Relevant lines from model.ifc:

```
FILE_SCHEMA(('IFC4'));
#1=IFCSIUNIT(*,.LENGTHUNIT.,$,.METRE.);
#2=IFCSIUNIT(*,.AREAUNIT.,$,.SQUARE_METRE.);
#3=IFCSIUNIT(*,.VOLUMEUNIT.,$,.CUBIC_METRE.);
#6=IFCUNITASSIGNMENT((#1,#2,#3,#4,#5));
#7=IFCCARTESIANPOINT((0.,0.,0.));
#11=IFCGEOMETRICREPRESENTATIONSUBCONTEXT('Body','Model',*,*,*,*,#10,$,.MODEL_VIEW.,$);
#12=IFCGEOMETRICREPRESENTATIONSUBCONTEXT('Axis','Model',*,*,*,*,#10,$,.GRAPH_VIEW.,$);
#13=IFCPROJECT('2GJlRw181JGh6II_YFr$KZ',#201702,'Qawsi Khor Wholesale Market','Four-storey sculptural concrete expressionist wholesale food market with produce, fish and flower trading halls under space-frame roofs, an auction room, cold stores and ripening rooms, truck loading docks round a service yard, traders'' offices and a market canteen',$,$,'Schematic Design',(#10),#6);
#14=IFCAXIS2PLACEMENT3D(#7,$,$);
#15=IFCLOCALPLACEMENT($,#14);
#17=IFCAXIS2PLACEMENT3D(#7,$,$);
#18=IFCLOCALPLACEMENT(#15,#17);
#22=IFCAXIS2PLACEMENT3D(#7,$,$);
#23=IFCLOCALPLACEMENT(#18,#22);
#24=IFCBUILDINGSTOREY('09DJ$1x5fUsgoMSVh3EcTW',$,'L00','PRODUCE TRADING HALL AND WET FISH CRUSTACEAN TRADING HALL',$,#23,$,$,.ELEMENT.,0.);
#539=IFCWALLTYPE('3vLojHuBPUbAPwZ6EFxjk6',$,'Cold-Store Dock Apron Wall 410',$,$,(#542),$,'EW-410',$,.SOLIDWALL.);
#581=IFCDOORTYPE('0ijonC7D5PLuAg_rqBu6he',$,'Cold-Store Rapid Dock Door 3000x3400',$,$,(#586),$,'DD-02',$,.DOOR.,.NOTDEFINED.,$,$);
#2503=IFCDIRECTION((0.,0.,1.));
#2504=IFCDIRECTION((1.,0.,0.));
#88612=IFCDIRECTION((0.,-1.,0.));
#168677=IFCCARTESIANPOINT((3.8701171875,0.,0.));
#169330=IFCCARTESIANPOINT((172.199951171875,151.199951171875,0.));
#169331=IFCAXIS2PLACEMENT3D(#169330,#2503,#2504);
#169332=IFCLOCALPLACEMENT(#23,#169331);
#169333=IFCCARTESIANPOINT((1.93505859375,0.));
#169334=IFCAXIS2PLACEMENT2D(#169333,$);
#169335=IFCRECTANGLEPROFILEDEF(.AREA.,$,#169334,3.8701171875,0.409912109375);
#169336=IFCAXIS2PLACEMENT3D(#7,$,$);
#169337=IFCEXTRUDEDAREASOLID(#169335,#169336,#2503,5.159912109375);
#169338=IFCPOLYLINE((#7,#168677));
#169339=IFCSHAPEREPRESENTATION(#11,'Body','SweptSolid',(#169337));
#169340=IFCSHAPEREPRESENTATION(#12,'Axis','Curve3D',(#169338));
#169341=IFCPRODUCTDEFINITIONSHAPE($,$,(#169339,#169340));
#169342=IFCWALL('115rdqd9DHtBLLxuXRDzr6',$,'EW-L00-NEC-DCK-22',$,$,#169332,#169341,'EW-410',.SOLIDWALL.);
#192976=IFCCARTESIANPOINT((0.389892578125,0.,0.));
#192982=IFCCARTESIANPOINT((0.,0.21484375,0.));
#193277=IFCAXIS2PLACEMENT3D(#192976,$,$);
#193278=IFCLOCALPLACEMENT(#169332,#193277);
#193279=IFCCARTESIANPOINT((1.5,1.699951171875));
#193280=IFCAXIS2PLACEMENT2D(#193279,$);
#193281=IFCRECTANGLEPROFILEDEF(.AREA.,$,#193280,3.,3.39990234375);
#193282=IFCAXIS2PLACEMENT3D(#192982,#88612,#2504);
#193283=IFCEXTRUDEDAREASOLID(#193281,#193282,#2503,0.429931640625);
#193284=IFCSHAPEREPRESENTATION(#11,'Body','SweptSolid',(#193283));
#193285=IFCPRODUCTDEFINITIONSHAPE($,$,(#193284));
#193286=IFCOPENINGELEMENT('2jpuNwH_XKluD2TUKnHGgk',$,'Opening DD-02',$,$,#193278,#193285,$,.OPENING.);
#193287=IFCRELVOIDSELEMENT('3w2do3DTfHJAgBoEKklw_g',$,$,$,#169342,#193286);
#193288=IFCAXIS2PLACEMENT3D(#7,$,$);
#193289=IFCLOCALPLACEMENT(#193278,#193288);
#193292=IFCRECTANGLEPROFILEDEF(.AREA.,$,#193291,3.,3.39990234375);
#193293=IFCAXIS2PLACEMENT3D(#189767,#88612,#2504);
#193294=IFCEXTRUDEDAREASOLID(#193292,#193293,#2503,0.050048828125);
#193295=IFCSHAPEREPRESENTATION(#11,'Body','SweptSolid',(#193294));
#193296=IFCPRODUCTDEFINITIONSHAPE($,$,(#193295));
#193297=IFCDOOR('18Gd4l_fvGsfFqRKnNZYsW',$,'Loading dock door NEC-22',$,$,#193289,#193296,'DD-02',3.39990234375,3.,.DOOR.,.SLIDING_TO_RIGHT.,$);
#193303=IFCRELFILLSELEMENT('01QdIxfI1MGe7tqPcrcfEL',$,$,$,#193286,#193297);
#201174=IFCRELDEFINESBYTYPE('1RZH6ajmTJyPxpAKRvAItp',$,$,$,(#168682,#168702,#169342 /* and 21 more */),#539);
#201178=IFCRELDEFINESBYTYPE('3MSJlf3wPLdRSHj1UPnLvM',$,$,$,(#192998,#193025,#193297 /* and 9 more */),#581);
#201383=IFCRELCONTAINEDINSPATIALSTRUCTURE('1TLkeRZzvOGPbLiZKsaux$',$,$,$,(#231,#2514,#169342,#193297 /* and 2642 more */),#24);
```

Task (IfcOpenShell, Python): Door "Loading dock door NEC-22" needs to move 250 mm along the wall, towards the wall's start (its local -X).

```python
import ifcopenshell
import ifcopenshell.api.geometry
import ifcopenshell.util.placement
import ifcopenshell.util.unit

model = ifcopenshell.open("model.ifc")
unit_scale = ifcopenshell.util.unit.calculate_unit_scale(model)

door = model.by_id(193297)
opening = door.FillsVoids[0].RelatingOpeningElement
wall = opening.VoidsElements[0].RelatingBuildingElement

wall_matrix = ifcopenshell.util.placement.get_local_placement(wall.ObjectPlacement)
shift = wall_matrix[:3, 0] * -0.25 / unit_scale
before = ifcopenshell.util.placement.get_local_placement(door.ObjectPlacement)[:3, 3].copy()

# The door is placed relative to its opening, so it follows when the opening moves.
matrix = ifcopenshell.util.placement.get_local_placement(opening.ObjectPlacement)
matrix[:3, 3] += shift
ifcopenshell.api.geometry.edit_object_placement(
    model, product=opening, matrix=matrix, is_si=False, should_transform_children=True
)

after = ifcopenshell.util.placement.get_local_placement(door.ObjectPlacement)[:3, 3]
print("door moved by", (after - before).round(3) + 0.0)

model.write("model-out.ifc")
```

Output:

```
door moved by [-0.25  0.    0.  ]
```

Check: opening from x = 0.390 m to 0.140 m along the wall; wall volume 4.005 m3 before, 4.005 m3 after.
